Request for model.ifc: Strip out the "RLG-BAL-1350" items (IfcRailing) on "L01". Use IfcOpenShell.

First a look at what the model holds.

```python
import ifcopenshell
import ifcopenshell.util.element

model = ifcopenshell.open("model.ifc")
print(model.schema)
storey = next(s for s in model.by_type("IfcBuildingStorey") if s.Name == "L01")
railings = [e for e in ifcopenshell.util.element.get_decomposition(storey) if e.is_a("IfcRailing")]
seen = {}
for e in railings:
    element_type = ifcopenshell.util.element.get_type(e)
    name = element_type.Name if element_type not in (None, e) else None
    seen[name] = seen.get(name, 0) + 1
for name, count in sorted(seen.items(), key=str):
    print(count, "x", name)
```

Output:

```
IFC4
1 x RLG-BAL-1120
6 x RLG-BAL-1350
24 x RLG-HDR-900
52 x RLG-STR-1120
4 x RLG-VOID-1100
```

```python
import ifcopenshell
import ifcopenshell.api.root
import ifcopenshell.util.element

model = ifcopenshell.open("model.ifc")

storey = next(s for s in model.by_type("IfcBuildingStorey") if s.Name == "L01")
railings = [e for e in ifcopenshell.util.element.get_decomposition(storey) if e.is_a("IfcRailing")]
targets = [e for e in railings if (t := ifcopenshell.util.element.get_type(e)) not in (None, e) and t.Name == "RLG-BAL-1350"]

for e in targets:
    ifcopenshell.api.root.remove_product(model, product=e)
print(len(targets), "removed")

model.write("model_edited.ifc")
```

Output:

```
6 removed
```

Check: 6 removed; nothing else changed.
